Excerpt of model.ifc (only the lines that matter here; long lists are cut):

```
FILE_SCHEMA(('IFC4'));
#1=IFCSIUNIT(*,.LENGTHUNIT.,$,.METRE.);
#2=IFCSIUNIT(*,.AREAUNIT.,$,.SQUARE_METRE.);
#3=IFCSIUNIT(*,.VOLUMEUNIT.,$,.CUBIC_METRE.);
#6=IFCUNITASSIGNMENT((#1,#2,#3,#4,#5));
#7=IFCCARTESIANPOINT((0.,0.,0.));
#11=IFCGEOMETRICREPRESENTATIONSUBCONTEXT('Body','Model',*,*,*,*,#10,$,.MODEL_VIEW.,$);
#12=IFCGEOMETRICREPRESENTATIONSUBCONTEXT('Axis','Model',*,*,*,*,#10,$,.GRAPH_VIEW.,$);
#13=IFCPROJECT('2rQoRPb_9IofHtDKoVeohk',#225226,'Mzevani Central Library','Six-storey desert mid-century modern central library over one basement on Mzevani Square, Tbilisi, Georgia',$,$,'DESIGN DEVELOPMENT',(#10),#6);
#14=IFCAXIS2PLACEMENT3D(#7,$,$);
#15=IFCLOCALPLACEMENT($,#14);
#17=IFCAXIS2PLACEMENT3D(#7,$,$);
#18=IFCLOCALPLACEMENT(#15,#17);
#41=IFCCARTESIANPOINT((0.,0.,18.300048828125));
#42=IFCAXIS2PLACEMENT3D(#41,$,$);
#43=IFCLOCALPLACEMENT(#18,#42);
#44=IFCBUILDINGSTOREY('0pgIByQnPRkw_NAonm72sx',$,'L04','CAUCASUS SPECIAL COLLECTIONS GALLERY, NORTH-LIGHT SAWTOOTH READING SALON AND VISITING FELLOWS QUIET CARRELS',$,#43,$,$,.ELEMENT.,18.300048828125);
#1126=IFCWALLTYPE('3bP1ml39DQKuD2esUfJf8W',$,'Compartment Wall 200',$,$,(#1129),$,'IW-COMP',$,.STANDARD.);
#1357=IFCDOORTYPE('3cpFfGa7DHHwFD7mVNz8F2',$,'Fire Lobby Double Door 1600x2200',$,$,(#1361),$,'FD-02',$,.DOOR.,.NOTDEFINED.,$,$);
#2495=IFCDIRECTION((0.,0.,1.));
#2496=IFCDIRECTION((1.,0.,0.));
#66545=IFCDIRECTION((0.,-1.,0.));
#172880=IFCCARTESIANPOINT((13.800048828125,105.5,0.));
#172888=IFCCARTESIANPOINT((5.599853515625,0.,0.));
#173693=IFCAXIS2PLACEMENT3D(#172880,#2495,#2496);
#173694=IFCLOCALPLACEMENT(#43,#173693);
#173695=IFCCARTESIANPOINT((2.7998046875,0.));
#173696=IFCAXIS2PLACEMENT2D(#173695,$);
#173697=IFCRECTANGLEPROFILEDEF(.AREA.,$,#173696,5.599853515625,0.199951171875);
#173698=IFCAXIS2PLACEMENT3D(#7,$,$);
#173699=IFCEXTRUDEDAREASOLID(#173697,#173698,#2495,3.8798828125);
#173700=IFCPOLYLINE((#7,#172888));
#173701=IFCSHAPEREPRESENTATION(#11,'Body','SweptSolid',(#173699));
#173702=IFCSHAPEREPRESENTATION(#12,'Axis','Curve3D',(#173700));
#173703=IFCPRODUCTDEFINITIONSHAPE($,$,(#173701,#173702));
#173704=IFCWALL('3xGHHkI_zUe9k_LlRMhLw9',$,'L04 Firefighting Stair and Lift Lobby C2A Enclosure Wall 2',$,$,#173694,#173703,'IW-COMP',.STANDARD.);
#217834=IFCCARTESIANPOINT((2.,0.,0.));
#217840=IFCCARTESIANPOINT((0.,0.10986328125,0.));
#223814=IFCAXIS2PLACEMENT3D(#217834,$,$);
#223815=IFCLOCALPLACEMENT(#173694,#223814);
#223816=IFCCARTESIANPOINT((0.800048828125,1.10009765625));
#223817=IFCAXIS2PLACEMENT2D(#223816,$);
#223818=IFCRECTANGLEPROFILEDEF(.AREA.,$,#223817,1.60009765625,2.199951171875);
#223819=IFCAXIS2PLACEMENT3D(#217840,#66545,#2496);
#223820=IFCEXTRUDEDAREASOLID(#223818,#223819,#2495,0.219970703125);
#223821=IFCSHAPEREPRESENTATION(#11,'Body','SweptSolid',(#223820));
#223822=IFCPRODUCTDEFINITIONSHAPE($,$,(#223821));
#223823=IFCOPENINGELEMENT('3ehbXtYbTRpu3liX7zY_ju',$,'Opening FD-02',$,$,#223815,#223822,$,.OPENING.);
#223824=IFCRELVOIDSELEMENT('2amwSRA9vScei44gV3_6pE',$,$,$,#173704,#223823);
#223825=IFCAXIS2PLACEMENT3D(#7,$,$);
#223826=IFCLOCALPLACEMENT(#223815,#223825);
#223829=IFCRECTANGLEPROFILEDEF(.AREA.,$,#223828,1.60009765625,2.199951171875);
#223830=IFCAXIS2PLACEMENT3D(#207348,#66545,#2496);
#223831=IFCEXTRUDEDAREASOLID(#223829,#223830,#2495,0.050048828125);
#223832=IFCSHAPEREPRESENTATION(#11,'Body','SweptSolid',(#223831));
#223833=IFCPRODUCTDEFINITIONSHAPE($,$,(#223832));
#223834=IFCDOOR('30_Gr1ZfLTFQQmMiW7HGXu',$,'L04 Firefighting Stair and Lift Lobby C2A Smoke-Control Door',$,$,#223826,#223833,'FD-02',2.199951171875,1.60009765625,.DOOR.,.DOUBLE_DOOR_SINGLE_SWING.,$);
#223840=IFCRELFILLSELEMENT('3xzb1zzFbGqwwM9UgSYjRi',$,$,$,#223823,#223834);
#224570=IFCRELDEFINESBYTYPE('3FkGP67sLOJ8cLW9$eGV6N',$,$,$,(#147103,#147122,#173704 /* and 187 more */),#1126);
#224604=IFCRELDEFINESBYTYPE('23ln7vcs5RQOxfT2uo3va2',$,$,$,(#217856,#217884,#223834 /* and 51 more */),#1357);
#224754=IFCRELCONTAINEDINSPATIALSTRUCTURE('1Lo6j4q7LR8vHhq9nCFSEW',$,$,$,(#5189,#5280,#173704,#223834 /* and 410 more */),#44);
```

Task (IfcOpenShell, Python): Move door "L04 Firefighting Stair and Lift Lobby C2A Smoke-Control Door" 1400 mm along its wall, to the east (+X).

```python
import ifcopenshell
import ifcopenshell.api.geometry
import ifcopenshell.util.placement
import ifcopenshell.util.unit

model = ifcopenshell.open("model.ifc")
unit_scale = ifcopenshell.util.unit.calculate_unit_scale(model)

door = model.by_id(223834)
opening = door.FillsVoids[0].RelatingOpeningElement
wall = opening.VoidsElements[0].RelatingBuildingElement

wall_matrix = ifcopenshell.util.placement.get_local_placement(wall.ObjectPlacement)
shift = wall_matrix[:3, 0] * 1.4 / unit_scale
before = ifcopenshell.util.placement.get_local_placement(door.ObjectPlacement)[:3, 3].copy()

# The door is placed relative to its opening, so it follows when the opening moves.
matrix = ifcopenshell.util.placement.get_local_placement(opening.ObjectPlacement)
matrix[:3, 3] += shift
ifcopenshell.api.geometry.edit_object_placement(
    model, product=opening, matrix=matrix, is_si=False, should_transform_children=True
)

after = ifcopenshell.util.placement.get_local_placement(door.ObjectPlacement)[:3, 3]
print("door moved by", (after - before).round(3) + 0.0)

model.write("model_v2.ifc")
```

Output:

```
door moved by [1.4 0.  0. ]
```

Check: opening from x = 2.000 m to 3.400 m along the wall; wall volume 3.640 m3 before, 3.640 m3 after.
